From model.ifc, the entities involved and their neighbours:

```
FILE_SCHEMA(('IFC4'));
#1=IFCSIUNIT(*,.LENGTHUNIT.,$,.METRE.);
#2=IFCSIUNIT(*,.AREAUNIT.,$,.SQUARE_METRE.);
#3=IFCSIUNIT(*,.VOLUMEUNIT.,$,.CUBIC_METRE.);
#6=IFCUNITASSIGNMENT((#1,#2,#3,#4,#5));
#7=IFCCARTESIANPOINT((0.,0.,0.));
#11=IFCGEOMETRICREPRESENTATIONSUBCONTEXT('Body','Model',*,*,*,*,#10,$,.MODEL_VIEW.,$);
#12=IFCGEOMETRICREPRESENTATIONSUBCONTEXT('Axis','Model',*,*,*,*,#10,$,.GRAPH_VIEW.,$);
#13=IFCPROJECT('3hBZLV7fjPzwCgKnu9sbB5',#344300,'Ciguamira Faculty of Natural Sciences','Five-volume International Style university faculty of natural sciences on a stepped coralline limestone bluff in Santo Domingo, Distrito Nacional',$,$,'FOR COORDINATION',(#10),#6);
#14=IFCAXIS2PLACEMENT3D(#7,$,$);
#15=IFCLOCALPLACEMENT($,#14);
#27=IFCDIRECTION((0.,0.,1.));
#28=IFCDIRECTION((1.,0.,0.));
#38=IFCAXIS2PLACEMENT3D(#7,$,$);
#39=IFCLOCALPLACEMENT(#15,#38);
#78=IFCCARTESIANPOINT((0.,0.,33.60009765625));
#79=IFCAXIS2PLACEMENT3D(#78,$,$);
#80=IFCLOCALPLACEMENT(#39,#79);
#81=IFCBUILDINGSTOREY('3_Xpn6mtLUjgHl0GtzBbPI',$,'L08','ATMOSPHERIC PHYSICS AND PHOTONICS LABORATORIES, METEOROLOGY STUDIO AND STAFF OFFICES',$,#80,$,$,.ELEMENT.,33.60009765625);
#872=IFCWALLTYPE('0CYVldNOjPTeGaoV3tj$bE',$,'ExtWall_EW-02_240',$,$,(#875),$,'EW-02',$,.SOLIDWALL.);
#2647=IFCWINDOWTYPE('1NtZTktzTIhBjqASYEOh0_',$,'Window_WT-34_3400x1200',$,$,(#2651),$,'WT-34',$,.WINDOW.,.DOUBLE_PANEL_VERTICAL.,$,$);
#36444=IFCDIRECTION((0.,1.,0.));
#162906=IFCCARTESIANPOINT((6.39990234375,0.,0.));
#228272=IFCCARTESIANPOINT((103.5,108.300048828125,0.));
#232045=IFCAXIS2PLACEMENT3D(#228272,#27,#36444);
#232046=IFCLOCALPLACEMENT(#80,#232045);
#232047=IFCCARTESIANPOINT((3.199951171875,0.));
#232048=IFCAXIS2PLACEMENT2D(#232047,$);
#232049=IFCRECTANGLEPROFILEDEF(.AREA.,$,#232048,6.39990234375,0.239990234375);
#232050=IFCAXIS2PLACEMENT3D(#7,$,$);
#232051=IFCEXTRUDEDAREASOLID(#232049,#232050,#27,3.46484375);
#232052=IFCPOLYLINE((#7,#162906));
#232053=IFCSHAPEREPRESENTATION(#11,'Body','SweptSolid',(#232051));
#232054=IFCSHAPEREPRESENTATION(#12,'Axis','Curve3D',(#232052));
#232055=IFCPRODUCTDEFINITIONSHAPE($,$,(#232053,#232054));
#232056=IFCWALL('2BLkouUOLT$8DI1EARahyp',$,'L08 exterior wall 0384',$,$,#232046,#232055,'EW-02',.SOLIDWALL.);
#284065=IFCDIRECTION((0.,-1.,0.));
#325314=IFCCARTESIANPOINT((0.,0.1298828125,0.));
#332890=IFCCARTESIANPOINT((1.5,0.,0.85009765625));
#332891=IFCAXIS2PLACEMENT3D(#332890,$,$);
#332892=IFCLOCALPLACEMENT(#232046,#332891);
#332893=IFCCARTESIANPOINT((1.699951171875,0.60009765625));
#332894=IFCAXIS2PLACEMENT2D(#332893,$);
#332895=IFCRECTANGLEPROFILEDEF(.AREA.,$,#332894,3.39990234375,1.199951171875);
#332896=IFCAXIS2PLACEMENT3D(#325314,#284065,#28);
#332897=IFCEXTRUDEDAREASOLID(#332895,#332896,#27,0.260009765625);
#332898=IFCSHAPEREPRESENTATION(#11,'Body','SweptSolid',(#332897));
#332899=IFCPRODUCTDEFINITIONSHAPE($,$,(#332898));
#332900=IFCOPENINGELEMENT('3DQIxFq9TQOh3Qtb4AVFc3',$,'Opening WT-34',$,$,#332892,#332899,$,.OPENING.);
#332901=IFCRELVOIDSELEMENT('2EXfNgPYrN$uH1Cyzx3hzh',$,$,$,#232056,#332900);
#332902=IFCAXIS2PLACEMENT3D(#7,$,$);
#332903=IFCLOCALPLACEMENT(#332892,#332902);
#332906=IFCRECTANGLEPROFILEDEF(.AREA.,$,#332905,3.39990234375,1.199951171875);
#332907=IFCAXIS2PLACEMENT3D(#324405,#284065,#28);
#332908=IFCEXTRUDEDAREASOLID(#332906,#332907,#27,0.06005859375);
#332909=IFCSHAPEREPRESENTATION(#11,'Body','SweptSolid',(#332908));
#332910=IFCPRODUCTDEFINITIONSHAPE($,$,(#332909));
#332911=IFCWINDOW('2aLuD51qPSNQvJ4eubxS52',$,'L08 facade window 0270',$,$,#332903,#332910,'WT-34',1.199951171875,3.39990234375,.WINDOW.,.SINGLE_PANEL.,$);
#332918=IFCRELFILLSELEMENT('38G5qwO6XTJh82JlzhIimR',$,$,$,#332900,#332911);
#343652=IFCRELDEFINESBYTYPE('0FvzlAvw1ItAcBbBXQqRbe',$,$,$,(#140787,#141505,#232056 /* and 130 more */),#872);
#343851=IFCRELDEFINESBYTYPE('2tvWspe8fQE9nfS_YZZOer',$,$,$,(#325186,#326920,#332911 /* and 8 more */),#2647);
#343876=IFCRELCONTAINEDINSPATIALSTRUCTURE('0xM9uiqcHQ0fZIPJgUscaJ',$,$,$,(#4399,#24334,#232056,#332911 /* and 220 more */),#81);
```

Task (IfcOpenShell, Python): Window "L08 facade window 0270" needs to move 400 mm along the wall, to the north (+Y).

```python
import ifcopenshell
import ifcopenshell.api.geometry
import ifcopenshell.util.placement
import ifcopenshell.util.unit

model = ifcopenshell.open("model.ifc")
unit_scale = ifcopenshell.util.unit.calculate_unit_scale(model)

window = model.by_guid("2aLuD51qPSNQvJ4eubxS52")
opening = window.FillsVoids[0].RelatingOpeningElement
wall = opening.VoidsElements[0].RelatingBuildingElement

wall_matrix = ifcopenshell.util.placement.get_local_placement(wall.ObjectPlacement)
shift = wall_matrix[:3, 0] * 0.4 / unit_scale
before = ifcopenshell.util.placement.get_local_placement(window.ObjectPlacement)[:3, 3].copy()

# The window is placed relative to its opening, so it follows when the opening moves.
matrix = ifcopenshell.util.placement.get_local_placement(opening.ObjectPlacement)
matrix[:3, 3] += shift
ifcopenshell.api.geometry.edit_object_placement(
    model, product=opening, matrix=matrix, is_si=False, should_transform_children=True
)

after = ifcopenshell.util.placement.get_local_placement(window.ObjectPlacement)[:3, 3]
print("window moved by", (after - before).round(3) + 0.0)

model.write("model_updated.ifc")
```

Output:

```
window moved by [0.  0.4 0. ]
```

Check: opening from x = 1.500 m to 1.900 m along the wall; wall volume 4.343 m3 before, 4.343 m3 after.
